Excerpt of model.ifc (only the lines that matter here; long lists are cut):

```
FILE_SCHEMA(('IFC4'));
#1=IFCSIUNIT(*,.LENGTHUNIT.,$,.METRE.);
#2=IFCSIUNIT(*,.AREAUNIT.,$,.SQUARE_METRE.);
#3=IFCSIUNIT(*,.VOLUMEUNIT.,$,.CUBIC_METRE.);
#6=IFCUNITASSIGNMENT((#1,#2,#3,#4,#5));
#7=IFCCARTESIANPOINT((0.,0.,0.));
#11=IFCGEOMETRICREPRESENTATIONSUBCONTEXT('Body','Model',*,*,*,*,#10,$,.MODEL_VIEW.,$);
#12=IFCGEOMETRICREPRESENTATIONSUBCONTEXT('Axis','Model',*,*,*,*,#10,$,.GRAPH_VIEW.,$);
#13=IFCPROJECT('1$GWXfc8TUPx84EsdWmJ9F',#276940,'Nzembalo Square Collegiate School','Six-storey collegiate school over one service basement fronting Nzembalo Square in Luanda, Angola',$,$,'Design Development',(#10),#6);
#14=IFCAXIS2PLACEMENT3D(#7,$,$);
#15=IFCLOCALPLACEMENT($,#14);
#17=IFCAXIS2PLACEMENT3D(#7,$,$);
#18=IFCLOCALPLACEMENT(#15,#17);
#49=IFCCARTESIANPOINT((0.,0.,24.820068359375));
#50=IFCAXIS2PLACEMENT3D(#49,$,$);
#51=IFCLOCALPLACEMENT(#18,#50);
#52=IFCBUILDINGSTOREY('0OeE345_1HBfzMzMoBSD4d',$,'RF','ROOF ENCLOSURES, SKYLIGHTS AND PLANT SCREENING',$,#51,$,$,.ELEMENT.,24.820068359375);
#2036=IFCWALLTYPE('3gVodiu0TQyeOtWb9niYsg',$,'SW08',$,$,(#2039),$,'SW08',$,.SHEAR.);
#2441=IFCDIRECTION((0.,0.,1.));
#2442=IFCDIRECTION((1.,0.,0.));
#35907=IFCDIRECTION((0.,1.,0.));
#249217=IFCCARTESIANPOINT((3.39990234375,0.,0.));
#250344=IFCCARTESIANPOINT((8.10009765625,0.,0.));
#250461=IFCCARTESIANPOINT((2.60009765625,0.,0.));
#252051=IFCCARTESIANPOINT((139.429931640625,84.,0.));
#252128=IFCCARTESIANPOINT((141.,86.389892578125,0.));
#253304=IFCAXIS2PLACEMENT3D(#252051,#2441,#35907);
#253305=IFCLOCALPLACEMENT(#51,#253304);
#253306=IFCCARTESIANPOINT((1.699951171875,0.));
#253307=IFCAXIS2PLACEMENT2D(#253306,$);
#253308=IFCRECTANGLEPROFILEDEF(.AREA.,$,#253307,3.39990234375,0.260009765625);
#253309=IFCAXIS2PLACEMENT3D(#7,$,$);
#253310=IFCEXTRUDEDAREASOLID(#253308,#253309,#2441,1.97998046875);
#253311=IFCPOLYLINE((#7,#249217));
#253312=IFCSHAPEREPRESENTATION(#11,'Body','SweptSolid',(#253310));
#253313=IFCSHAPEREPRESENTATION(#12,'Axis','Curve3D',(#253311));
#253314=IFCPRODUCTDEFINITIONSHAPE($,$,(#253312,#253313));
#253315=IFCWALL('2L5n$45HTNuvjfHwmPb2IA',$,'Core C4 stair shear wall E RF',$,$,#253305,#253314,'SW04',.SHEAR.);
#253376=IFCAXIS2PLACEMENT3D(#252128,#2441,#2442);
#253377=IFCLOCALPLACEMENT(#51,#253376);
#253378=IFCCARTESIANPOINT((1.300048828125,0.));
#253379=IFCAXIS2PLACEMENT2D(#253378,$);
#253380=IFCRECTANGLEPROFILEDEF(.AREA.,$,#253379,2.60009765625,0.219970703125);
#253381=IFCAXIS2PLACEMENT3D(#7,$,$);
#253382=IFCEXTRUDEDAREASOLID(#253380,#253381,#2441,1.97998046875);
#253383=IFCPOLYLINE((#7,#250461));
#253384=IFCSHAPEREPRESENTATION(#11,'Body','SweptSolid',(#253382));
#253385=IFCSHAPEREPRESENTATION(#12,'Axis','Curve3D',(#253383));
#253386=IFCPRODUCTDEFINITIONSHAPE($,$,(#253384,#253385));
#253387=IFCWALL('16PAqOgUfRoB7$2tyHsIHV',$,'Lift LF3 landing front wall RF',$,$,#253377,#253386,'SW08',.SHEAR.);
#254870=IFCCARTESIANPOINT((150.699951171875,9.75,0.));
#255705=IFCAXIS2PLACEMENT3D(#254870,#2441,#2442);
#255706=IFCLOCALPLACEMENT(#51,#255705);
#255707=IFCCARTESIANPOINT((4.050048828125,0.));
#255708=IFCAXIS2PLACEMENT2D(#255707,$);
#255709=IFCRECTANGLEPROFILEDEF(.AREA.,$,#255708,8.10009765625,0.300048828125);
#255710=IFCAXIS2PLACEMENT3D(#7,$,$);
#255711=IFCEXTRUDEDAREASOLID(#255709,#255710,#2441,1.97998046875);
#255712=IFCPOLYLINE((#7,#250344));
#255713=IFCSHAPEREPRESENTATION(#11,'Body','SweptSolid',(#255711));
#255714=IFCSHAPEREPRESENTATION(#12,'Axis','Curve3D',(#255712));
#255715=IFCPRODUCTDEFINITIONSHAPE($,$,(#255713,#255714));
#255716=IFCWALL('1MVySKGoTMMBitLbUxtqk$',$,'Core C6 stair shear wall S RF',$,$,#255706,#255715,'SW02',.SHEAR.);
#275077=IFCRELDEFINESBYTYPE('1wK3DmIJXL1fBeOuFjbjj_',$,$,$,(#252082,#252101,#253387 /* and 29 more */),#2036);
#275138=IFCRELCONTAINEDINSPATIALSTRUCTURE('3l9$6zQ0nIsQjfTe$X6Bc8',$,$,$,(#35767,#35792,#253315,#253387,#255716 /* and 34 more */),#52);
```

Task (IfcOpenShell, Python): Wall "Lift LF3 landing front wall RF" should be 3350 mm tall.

```python
import ifcopenshell
import ifcopenshell.geom
import ifcopenshell.util.representation
import ifcopenshell.util.shape
import ifcopenshell.util.unit

model = ifcopenshell.open("model.ifc")
unit_scale = ifcopenshell.util.unit.calculate_unit_scale(model)
settings = ifcopenshell.geom.settings()


def volume(element):
    """Net volume in cubic metres, openings subtracted."""
    shape = ifcopenshell.geom.create_shape(settings, element)
    return ifcopenshell.util.shape.get_volume(shape.geometry)


wall = model.by_guid("16PAqOgUfRoB7$2tyHsIHV")
before = volume(wall)

body = ifcopenshell.util.representation.get_representation(wall, "Model", "Body")
solid = body.Items[0]
old_height = solid.Depth
solid.Depth = 3.35 / unit_scale
after = volume(wall)

print(f"height {old_height:g} -> {solid.Depth:g}, volume {before:.3f} -> {after:.3f} m3")

model.write("model_updated.ifc")
```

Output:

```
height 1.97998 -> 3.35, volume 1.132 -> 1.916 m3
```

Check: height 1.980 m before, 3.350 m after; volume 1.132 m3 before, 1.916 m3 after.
